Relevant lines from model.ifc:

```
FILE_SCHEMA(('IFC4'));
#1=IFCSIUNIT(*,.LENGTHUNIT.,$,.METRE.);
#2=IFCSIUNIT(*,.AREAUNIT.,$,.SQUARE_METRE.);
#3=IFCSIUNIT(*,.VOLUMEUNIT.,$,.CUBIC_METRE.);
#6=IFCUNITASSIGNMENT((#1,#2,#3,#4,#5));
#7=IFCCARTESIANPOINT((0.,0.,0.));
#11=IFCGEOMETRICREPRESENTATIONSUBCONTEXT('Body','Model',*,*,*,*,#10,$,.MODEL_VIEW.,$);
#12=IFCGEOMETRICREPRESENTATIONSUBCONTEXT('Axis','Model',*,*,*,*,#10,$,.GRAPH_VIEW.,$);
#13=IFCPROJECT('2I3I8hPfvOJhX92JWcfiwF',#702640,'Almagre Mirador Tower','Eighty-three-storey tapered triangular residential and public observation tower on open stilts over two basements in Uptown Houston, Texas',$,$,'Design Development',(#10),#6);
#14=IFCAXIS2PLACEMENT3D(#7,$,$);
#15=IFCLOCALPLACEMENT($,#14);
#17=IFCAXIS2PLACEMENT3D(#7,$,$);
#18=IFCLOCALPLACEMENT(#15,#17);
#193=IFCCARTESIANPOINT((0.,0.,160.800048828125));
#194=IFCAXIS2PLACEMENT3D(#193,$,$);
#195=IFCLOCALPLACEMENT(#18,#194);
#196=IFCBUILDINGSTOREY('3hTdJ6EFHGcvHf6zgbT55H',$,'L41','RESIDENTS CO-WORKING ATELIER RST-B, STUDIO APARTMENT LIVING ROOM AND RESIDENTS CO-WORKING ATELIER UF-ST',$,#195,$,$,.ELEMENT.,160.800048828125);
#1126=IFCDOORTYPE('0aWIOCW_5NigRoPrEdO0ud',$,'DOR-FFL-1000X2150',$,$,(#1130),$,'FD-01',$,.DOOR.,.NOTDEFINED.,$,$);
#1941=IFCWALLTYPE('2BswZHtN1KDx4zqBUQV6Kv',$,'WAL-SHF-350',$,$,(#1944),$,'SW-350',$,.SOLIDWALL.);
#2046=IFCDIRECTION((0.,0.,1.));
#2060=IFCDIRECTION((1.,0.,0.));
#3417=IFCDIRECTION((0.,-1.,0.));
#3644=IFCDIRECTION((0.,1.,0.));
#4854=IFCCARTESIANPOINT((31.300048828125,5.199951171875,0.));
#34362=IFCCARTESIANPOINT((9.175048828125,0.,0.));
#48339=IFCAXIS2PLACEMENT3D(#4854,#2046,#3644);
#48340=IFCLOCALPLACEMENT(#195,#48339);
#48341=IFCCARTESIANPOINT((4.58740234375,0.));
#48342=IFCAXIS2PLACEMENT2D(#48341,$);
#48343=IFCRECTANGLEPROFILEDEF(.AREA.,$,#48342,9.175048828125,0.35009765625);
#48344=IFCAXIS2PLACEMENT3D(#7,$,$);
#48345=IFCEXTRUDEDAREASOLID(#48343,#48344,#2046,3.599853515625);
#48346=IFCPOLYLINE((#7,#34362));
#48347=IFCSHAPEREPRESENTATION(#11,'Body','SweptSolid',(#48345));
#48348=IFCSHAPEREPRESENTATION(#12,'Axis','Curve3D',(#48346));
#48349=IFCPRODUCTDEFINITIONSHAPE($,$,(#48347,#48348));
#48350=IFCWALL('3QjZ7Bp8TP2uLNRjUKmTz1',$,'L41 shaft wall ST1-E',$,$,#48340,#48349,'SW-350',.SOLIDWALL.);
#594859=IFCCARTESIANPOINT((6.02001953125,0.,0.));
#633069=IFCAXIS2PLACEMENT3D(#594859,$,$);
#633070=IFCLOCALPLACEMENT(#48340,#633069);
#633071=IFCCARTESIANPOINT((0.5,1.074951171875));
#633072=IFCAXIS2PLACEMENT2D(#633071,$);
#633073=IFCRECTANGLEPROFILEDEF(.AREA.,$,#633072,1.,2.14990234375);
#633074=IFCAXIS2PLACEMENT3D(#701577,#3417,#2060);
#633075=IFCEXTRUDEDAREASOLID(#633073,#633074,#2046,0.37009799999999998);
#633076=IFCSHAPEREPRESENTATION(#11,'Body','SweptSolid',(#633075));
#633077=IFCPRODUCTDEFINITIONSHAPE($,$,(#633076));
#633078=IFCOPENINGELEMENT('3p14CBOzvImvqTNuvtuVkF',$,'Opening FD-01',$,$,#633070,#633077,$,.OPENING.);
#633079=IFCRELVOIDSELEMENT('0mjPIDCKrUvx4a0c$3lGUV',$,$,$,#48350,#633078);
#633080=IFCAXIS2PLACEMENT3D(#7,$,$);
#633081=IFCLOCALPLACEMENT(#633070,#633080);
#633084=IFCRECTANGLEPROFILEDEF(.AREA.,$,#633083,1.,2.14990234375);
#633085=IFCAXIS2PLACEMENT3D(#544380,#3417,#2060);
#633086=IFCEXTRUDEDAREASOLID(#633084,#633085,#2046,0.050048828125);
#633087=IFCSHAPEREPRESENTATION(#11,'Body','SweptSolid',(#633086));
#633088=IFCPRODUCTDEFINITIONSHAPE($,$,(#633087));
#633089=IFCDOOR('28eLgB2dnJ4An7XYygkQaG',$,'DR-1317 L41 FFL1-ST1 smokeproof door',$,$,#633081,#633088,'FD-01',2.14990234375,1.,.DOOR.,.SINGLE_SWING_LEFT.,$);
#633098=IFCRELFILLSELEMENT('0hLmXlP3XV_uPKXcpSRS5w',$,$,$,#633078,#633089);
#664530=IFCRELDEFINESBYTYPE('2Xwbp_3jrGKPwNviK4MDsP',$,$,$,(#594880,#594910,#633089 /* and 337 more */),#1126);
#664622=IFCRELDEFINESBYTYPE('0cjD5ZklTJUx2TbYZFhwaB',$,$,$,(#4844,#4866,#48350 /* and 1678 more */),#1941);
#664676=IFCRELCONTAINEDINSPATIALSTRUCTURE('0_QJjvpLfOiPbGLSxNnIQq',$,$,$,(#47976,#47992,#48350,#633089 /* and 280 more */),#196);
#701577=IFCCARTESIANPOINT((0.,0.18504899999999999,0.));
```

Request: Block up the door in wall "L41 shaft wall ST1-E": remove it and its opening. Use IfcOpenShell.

```python
import ifcopenshell
import ifcopenshell.api.feature
import ifcopenshell.api.root
import ifcopenshell.geom
import ifcopenshell.util.shape

model = ifcopenshell.open("model.ifc")
settings = ifcopenshell.geom.settings()


def volume(element):
    """Net volume in cubic metres, openings subtracted."""
    shape = ifcopenshell.geom.create_shape(settings, element)
    return ifcopenshell.util.shape.get_volume(shape.geometry)


door = model.by_id(633089)
opening = door.FillsVoids[0].RelatingOpeningElement
wall = opening.VoidsElements[0].RelatingBuildingElement
before = volume(wall)

ifcopenshell.api.root.remove_product(model, product=door)
ifcopenshell.api.feature.remove_feature(model, feature=opening)

after = volume(wall)

print(f"wall volume {before:.3f} -> {after:.3f} m3")

model.write("model_rev.ifc")
```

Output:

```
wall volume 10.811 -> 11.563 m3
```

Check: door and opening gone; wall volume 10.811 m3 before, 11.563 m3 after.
